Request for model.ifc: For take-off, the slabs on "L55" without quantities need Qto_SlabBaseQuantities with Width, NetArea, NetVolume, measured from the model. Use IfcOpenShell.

First a look at what the model holds.

```python
import ifcopenshell
import ifcopenshell.util.element
import ifcopenshell.util.unit

model = ifcopenshell.open("model.ifc")
print(model.schema)
for unit_type in ("LENGTHUNIT", "AREAUNIT", "VOLUMEUNIT"):
    print(unit_type, ifcopenshell.util.unit.calculate_unit_scale(model, unit_type))
storey = next(s for s in model.by_type("IfcBuildingStorey") if s.Name == "L55")
slabs = [e for e in ifcopenshell.util.element.get_decomposition(storey) if e.is_a("IfcSlab")]
for e in sorted(slabs, key=lambda e: e.id()):
    print(e.id(), e.is_a(), e.Name, list(ifcopenshell.util.element.get_psets(e, qtos_only=True)), sep=" | ")
```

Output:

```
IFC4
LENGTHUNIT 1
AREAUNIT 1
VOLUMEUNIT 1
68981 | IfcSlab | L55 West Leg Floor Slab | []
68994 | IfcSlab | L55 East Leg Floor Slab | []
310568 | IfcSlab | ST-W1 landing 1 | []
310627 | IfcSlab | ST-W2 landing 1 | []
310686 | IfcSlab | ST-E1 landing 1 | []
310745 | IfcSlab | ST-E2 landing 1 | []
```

```python
import ifcopenshell
import ifcopenshell.api.pset
import ifcopenshell.geom
import ifcopenshell.util.element
import ifcopenshell.util.shape
import ifcopenshell.util.unit

model = ifcopenshell.open("model.ifc")
unit_scale = ifcopenshell.util.unit.calculate_unit_scale(model)
area_scale = ifcopenshell.util.unit.calculate_unit_scale(model, "AREAUNIT")
volume_scale = ifcopenshell.util.unit.calculate_unit_scale(model, "VOLUMEUNIT")
settings = ifcopenshell.geom.settings()

storey = next(s for s in model.by_type("IfcBuildingStorey") if s.Name == "L55")
slabs = [e for e in ifcopenshell.util.element.get_decomposition(storey) if e.is_a("IfcSlab")]

for e in sorted(slabs, key=lambda e: e.id()):
    if ifcopenshell.util.element.get_psets(e, qtos_only=True, should_inherit=False):
        continue
    # Geometry comes back in metres, in the element's own axes.
    shape = ifcopenshell.geom.create_shape(settings, e)
    values = {
        "Width": ifcopenshell.util.shape.get_z(shape.geometry) / unit_scale,
        "NetArea": ifcopenshell.util.shape.get_footprint_area(shape.geometry) / area_scale,
        "NetVolume": ifcopenshell.util.shape.get_volume(shape.geometry) / volume_scale,
    }
    qto = ifcopenshell.api.pset.add_qto(model, product=e, name="Qto_SlabBaseQuantities")
    ifcopenshell.api.pset.edit_qto(model, qto=qto, properties=values)
    print(e.id(), {k: round(v, 3) for k, v in values.items()})

model.write("model_v2.ifc")
```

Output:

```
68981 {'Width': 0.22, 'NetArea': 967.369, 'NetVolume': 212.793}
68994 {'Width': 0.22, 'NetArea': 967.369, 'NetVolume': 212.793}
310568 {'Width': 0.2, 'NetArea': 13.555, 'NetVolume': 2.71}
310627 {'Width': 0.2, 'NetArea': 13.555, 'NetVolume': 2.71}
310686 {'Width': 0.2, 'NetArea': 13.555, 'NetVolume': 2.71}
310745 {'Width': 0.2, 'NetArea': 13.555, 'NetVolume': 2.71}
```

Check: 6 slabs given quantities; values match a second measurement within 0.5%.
